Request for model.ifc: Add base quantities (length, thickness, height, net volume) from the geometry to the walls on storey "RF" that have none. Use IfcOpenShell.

First a look at what the model holds.

```python
import ifcopenshell
import ifcopenshell.util.element
import ifcopenshell.util.unit

model = ifcopenshell.open("model.ifc")
print(model.schema)
for unit_type in ("LENGTHUNIT", "AREAUNIT", "VOLUMEUNIT"):
    print(unit_type, ifcopenshell.util.unit.calculate_unit_scale(model, unit_type))
storey = next(s for s in model.by_type("IfcBuildingStorey") if s.Name == "RF")
walls = [e for e in ifcopenshell.util.element.get_decomposition(storey) if e.is_a("IfcWall")]
for e in sorted(walls, key=lambda e: e.id()):
    print(e.id(), e.is_a(), e.Name, list(ifcopenshell.util.element.get_psets(e, qtos_only=True)), sep=" | ")
```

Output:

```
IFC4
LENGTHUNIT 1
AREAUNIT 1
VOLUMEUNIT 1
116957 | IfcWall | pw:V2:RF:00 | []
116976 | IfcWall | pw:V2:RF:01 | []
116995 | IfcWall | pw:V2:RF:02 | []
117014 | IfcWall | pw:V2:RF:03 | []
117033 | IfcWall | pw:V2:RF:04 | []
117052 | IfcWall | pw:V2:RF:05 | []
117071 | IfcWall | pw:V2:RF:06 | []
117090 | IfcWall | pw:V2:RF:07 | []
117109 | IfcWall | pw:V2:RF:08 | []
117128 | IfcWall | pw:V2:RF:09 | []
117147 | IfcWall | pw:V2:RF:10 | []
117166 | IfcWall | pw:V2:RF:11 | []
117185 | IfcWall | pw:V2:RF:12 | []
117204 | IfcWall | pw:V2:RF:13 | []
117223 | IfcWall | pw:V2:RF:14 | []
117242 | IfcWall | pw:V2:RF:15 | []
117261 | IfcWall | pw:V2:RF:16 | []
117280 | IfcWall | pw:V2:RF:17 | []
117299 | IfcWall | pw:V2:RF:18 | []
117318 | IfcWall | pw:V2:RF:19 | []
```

```python
import ifcopenshell
import ifcopenshell.api.pset
import ifcopenshell.geom
import ifcopenshell.util.element
import ifcopenshell.util.shape
import ifcopenshell.util.unit

model = ifcopenshell.open("model.ifc")
unit_scale = ifcopenshell.util.unit.calculate_unit_scale(model)
volume_scale = ifcopenshell.util.unit.calculate_unit_scale(model, "VOLUMEUNIT")
settings = ifcopenshell.geom.settings()

storey = next(s for s in model.by_type("IfcBuildingStorey") if s.Name == "RF")
walls = [e for e in ifcopenshell.util.element.get_decomposition(storey) if e.is_a("IfcWall")]

for e in sorted(walls, key=lambda e: e.id()):
    if ifcopenshell.util.element.get_psets(e, qtos_only=True, should_inherit=False):
        continue
    # Geometry comes back in metres, in the element's own axes.
    shape = ifcopenshell.geom.create_shape(settings, e)
    values = {
        "Length": ifcopenshell.util.shape.get_x(shape.geometry) / unit_scale,
        "Width": ifcopenshell.util.shape.get_y(shape.geometry) / unit_scale,
        "Height": ifcopenshell.util.shape.get_z(shape.geometry) / unit_scale,
        "NetVolume": ifcopenshell.util.shape.get_volume(shape.geometry) / volume_scale,
    }
    qto = ifcopenshell.api.pset.add_qto(model, product=e, name="Qto_WallBaseQuantities")
    ifcopenshell.api.pset.edit_qto(model, qto=qto, properties=values)
    print(e.id(), {k: round(v, 3) for k, v in values.items()})

model.write("model-out.ifc")
```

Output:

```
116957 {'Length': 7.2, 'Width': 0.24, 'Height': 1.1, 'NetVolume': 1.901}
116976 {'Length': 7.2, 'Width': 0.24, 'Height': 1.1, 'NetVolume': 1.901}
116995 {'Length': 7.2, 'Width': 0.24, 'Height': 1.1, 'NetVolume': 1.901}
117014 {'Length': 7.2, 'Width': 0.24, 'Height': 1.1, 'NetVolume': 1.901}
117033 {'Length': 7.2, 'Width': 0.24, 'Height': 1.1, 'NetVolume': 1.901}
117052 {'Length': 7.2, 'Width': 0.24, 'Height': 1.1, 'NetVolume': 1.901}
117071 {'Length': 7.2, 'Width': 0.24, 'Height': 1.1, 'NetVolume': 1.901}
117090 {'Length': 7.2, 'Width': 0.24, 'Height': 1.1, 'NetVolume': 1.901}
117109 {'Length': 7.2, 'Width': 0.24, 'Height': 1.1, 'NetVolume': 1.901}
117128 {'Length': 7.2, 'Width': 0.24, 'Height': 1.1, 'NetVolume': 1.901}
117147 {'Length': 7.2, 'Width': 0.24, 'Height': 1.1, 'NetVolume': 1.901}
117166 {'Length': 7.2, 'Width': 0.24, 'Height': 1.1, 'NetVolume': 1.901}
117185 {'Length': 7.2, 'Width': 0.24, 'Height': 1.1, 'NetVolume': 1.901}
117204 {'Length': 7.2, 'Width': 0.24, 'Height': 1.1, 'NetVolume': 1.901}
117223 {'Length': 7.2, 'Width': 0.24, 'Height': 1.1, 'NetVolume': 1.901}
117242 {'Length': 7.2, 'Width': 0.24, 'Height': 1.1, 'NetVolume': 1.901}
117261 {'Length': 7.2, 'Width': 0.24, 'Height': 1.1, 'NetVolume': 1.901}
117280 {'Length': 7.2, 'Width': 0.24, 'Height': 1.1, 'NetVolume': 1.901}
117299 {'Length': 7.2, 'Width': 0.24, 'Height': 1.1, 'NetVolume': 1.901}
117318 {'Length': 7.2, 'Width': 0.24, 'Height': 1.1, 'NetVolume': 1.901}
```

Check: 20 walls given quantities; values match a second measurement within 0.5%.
